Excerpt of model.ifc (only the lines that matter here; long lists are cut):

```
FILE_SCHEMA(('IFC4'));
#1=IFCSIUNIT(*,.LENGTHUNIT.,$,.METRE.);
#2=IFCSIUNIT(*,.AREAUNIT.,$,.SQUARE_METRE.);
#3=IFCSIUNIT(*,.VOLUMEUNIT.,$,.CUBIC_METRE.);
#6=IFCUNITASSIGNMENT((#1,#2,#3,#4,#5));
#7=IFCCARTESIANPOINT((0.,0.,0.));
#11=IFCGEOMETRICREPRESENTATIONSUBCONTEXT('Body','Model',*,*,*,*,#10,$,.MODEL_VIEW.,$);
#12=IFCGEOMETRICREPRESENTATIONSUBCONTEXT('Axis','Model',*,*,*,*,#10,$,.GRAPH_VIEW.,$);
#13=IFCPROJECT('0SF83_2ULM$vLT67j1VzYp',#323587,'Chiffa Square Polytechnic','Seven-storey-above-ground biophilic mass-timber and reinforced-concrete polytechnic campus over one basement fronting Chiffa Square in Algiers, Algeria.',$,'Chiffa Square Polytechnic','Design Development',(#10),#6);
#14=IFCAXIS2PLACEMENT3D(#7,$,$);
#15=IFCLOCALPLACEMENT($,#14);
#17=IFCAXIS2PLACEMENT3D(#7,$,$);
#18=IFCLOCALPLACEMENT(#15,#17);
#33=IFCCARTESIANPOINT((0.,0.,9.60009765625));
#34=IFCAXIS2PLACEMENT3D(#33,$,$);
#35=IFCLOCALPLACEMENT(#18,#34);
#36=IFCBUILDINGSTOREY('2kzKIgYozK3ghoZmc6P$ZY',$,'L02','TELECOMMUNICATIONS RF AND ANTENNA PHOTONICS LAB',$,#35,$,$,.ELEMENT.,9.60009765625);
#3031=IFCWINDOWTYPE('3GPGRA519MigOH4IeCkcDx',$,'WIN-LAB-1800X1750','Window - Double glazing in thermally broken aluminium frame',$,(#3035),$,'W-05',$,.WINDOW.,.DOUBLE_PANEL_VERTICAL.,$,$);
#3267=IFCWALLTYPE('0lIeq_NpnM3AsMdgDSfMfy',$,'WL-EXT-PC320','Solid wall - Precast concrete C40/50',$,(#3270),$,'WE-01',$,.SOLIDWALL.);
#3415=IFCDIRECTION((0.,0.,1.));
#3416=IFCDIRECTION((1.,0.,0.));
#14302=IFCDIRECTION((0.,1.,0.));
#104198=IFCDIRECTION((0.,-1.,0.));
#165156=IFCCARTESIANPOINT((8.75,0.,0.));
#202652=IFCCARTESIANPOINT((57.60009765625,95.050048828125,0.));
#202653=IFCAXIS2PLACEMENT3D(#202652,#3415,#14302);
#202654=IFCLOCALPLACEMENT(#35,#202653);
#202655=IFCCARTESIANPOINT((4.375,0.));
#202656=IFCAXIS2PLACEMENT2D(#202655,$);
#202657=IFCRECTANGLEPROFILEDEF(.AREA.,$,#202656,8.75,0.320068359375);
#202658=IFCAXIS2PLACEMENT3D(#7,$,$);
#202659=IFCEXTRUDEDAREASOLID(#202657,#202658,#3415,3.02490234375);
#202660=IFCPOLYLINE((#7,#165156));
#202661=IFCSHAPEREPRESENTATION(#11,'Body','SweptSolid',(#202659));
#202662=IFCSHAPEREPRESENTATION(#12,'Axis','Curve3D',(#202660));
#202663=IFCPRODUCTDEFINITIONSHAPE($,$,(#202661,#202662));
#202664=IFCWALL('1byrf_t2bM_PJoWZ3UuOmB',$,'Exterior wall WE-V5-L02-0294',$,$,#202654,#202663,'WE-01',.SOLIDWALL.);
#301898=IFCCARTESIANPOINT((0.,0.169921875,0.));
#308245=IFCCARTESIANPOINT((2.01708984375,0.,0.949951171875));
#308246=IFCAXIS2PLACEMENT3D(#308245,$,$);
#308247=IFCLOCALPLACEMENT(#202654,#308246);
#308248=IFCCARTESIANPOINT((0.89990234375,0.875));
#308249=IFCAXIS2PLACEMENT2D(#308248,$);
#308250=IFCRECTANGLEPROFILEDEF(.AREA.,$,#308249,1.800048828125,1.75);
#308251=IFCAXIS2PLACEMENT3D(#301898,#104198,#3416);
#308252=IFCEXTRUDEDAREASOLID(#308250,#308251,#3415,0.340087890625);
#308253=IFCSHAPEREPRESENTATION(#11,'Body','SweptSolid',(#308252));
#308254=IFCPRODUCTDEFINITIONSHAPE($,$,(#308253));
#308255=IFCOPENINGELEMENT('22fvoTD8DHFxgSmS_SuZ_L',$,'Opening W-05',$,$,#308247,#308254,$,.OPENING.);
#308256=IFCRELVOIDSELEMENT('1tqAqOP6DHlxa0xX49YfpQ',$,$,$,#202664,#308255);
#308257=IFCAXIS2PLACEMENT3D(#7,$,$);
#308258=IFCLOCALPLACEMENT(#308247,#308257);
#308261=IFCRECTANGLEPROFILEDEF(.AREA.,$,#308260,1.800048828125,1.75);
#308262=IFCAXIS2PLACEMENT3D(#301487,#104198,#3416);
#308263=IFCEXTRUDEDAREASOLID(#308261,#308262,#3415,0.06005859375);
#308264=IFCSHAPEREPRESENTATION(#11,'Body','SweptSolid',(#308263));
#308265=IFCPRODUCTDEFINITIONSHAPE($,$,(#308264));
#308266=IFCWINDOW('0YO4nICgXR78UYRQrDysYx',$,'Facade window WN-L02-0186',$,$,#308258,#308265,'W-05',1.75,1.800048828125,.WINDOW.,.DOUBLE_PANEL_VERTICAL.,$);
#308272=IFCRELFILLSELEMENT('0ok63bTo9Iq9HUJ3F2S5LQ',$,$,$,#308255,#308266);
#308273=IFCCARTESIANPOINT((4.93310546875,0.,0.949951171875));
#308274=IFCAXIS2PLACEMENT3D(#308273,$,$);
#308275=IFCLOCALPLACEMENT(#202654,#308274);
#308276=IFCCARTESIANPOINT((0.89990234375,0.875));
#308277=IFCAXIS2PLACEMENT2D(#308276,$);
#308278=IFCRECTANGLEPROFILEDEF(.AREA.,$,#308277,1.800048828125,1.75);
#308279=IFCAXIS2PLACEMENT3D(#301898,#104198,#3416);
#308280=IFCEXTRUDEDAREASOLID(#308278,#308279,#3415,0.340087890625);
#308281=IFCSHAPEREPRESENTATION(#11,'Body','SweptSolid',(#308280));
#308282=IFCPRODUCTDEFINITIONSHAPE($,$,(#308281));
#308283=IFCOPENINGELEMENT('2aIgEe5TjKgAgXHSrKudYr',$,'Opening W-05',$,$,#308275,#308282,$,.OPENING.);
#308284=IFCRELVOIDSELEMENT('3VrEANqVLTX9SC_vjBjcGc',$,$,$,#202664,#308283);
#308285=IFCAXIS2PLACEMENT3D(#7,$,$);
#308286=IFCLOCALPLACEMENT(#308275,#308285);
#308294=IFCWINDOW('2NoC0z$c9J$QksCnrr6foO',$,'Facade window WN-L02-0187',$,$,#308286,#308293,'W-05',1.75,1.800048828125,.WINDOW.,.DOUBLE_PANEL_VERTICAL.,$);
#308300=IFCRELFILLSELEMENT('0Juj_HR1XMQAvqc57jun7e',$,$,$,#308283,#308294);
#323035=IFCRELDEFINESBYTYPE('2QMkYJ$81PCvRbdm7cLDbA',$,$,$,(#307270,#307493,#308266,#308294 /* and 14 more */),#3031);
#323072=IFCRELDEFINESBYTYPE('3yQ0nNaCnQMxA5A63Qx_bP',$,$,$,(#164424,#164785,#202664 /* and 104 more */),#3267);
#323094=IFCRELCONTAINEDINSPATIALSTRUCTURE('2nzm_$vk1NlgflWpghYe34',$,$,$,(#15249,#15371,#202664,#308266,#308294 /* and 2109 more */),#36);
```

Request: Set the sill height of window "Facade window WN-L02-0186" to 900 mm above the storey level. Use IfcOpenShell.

```python
import numpy as np
import ifcopenshell
import ifcopenshell.api.geometry
import ifcopenshell.geom
import ifcopenshell.util.element
import ifcopenshell.util.placement
import ifcopenshell.util.shape
import ifcopenshell.util.unit

model = ifcopenshell.open("model.ifc")
unit_scale = ifcopenshell.util.unit.calculate_unit_scale(model)

window = model.by_guid("0YO4nICgXR78UYRQrDysYx")
opening = window.FillsVoids[0].RelatingOpeningElement
storey = ifcopenshell.util.element.get_container(window, ifc_class="IfcBuildingStorey")
level = ifcopenshell.util.placement.get_local_placement(storey.ObjectPlacement)[2, 3]

# The opening's origin need not be at the sill, so measure its lowest point.
shape = ifcopenshell.geom.create_shape(ifcopenshell.geom.settings(), opening)
bottom = ifcopenshell.util.shape.get_shape_bottom_elevation(shape, shape.geometry) / unit_scale
dz = level + 0.9 / unit_scale - bottom

shift = np.array([0.0, 0.0, dz])
# The window is placed relative to its opening, so it follows when the opening moves.
matrix = ifcopenshell.util.placement.get_local_placement(opening.ObjectPlacement)
matrix[:3, 3] += shift
ifcopenshell.api.geometry.edit_object_placement(
    model, product=opening, matrix=matrix, is_si=False, should_transform_children=True
)

print(f"moved by {dz * unit_scale:+.3f} m")

model.write("model_edited.ifc")
```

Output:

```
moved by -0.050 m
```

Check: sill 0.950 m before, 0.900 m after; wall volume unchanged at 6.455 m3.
